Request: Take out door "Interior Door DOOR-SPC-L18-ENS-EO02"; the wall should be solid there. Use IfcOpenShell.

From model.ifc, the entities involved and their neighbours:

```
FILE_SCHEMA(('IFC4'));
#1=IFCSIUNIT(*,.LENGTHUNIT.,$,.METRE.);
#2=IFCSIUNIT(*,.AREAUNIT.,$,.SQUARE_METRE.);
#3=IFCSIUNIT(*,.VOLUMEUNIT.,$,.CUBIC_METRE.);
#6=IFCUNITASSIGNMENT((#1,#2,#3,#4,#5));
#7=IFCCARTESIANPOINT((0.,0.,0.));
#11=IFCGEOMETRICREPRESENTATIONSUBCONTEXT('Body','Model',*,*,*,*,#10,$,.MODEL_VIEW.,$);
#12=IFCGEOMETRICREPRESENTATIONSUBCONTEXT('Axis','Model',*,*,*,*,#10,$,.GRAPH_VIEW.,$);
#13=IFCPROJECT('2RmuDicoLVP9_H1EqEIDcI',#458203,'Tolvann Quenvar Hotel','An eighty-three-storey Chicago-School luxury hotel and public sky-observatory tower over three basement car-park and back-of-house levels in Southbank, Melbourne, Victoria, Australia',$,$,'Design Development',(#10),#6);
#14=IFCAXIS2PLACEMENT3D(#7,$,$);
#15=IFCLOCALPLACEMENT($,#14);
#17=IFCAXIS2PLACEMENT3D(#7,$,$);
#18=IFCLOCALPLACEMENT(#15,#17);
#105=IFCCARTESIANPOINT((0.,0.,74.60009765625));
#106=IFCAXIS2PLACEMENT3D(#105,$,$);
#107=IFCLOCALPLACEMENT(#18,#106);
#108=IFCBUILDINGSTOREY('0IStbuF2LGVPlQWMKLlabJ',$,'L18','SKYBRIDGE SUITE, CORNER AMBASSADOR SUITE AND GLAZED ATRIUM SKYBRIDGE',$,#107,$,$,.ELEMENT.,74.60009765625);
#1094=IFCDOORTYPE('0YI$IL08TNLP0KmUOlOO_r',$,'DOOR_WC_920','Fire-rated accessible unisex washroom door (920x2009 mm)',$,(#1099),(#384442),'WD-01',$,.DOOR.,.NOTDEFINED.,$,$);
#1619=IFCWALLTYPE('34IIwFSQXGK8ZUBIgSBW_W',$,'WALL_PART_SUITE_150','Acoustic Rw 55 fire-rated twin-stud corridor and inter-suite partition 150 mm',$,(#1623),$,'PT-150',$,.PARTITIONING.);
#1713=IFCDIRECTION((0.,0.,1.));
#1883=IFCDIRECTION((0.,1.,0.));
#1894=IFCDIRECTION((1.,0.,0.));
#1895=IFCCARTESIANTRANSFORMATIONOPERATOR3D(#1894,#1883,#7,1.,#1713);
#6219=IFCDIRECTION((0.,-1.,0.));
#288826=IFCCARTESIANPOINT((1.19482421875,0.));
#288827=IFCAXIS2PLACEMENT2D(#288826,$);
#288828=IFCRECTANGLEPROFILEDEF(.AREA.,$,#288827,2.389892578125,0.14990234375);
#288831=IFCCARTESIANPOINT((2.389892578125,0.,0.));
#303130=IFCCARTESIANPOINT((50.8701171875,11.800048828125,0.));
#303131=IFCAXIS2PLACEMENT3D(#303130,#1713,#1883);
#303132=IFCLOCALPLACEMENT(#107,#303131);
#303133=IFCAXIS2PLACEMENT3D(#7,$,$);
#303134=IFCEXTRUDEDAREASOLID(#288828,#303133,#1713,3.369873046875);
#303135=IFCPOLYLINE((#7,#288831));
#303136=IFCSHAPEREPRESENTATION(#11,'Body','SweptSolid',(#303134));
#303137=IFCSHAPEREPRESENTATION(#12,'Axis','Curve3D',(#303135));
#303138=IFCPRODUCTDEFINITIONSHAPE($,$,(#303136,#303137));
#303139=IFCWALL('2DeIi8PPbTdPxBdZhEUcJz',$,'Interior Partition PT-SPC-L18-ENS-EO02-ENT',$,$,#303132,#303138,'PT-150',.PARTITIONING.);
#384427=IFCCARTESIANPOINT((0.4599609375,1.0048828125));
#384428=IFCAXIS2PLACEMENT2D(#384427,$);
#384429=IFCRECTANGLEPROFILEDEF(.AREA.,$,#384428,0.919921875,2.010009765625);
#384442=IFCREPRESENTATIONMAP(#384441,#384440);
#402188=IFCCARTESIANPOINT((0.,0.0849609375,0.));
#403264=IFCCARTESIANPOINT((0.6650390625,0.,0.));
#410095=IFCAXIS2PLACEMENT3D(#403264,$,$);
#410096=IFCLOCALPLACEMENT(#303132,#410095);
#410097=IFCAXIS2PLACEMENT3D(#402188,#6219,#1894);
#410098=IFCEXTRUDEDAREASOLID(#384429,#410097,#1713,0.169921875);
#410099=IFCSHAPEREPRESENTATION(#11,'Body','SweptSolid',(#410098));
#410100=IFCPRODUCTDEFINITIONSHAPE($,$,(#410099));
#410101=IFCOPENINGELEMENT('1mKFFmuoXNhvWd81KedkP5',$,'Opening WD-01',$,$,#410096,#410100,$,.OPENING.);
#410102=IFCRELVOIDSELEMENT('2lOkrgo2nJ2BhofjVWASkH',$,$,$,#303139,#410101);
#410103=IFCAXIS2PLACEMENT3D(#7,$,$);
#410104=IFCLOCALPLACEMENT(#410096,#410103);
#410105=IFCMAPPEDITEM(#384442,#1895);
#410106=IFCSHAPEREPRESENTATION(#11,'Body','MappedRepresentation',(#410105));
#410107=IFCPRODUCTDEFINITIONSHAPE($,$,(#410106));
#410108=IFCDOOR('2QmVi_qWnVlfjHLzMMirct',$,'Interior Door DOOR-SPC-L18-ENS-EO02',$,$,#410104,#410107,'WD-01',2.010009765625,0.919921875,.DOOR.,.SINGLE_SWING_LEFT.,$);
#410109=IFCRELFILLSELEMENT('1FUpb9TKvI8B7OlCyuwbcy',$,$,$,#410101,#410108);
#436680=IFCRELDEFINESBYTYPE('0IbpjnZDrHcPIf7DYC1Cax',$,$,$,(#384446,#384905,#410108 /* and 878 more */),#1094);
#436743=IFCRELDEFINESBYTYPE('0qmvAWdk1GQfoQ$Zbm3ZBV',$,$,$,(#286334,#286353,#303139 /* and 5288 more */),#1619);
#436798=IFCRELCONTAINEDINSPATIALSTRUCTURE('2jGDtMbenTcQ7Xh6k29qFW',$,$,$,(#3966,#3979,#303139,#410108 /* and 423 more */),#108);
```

```python
import ifcopenshell
import ifcopenshell.api.feature
import ifcopenshell.api.root
import ifcopenshell.geom
import ifcopenshell.util.shape

model = ifcopenshell.open("model.ifc")
settings = ifcopenshell.geom.settings()


def volume(element):
    """Net volume in cubic metres, openings subtracted."""
    shape = ifcopenshell.geom.create_shape(settings, element)
    return ifcopenshell.util.shape.get_volume(shape.geometry)


door = model.by_guid("2QmVi_qWnVlfjHLzMMirct")
opening = door.FillsVoids[0].RelatingOpeningElement
wall = opening.VoidsElements[0].RelatingBuildingElement
before = volume(wall)

ifcopenshell.api.root.remove_product(model, product=door)
ifcopenshell.api.feature.remove_feature(model, feature=opening)

after = volume(wall)

print(f"wall volume {before:.3f} -> {after:.3f} m3")

model.write("model_edited.ifc")
```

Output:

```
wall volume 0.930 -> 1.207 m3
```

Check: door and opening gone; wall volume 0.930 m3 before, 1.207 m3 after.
